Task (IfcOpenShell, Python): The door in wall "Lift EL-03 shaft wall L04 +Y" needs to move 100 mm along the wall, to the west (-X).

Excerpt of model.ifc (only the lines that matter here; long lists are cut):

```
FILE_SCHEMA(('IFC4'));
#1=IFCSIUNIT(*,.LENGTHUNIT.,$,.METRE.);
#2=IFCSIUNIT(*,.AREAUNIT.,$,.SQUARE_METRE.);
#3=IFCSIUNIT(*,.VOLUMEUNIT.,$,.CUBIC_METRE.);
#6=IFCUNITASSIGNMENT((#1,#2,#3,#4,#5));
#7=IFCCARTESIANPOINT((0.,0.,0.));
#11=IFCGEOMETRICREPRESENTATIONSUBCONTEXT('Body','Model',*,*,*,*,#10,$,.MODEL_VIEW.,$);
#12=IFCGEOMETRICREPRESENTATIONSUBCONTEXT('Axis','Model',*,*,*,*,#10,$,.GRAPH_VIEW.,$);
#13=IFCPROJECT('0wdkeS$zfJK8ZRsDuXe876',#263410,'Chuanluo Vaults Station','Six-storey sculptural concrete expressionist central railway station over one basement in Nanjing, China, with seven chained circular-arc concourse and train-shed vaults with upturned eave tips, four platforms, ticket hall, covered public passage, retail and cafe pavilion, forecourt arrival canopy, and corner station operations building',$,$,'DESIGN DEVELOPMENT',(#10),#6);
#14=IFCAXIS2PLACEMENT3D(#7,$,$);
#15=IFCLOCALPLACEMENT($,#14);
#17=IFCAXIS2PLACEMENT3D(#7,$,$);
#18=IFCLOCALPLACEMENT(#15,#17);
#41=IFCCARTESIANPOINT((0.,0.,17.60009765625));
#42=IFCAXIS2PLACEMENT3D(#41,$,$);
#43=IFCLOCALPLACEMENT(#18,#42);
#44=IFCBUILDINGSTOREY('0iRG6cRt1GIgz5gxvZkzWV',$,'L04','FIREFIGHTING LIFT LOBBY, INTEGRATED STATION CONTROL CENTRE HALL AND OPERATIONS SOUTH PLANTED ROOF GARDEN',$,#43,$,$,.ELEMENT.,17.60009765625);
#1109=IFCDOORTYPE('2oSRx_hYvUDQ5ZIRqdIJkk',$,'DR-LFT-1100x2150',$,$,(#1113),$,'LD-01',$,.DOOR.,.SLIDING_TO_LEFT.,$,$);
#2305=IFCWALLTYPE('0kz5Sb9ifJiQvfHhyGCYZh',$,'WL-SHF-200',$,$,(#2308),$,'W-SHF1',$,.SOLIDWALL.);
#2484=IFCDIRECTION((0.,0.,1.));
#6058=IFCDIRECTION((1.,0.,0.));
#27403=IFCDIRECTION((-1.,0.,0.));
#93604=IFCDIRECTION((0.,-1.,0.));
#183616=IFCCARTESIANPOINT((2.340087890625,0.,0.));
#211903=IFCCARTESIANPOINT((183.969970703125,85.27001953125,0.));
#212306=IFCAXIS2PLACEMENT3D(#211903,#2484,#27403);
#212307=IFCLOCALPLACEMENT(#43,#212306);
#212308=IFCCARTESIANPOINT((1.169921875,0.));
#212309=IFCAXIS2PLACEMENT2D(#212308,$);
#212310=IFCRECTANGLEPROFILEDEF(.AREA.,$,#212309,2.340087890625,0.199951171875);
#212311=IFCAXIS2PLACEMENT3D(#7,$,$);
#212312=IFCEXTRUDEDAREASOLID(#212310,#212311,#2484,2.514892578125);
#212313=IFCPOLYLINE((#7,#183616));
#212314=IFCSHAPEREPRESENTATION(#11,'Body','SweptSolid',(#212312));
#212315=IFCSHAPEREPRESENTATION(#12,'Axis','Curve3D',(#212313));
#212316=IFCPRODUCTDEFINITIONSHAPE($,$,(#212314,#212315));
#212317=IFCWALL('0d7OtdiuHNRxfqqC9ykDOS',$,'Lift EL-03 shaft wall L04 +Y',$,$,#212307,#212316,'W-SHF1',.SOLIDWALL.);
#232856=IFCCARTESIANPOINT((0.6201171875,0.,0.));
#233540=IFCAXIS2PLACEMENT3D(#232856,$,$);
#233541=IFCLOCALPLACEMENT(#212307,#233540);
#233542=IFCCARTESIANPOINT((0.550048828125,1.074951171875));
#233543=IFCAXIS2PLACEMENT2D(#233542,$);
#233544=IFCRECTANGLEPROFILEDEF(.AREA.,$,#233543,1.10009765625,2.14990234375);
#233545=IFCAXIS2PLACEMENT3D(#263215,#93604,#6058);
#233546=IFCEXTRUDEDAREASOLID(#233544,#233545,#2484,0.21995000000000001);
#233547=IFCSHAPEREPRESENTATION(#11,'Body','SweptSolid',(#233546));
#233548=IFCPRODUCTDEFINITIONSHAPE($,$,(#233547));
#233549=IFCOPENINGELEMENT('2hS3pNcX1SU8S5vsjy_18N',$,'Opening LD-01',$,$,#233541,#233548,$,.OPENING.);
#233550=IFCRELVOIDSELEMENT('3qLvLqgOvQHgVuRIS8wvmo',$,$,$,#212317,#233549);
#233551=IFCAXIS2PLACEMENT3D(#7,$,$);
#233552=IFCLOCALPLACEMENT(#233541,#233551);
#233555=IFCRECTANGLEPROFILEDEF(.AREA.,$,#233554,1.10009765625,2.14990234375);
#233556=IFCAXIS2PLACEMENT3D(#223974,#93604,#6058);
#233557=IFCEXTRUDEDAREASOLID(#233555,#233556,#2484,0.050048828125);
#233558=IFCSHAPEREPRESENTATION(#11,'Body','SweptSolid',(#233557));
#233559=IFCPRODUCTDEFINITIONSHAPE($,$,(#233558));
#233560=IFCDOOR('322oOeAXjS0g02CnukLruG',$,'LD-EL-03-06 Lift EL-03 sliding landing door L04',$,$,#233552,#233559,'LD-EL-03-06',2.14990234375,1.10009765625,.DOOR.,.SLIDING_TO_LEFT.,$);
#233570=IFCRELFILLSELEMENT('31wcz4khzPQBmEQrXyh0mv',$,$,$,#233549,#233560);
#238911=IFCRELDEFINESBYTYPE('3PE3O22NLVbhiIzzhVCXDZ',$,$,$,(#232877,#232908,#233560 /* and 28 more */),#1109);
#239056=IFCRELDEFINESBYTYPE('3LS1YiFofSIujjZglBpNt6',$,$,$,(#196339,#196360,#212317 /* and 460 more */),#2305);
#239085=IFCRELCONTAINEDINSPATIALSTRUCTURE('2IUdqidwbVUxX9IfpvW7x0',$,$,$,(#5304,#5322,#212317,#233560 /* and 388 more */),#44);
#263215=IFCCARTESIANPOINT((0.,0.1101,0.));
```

```python
import ifcopenshell
import ifcopenshell.api.geometry
import ifcopenshell.util.placement
import ifcopenshell.util.unit

model = ifcopenshell.open("model.ifc")
unit_scale = ifcopenshell.util.unit.calculate_unit_scale(model)

door = model.by_guid("322oOeAXjS0g02CnukLruG")
opening = door.FillsVoids[0].RelatingOpeningElement
wall = opening.VoidsElements[0].RelatingBuildingElement

wall_matrix = ifcopenshell.util.placement.get_local_placement(wall.ObjectPlacement)
shift = wall_matrix[:3, 0] * 0.1 / unit_scale
before = ifcopenshell.util.placement.get_local_placement(door.ObjectPlacement)[:3, 3].copy()

# The door is placed relative to its opening, so it follows when the opening moves.
matrix = ifcopenshell.util.placement.get_local_placement(opening.ObjectPlacement)
matrix[:3, 3] += shift
ifcopenshell.api.geometry.edit_object_placement(
    model, product=opening, matrix=matrix, is_si=False, should_transform_children=True
)

after = ifcopenshell.util.placement.get_local_placement(door.ObjectPlacement)[:3, 3]
print("door moved by", (after - before).round(3) + 0.0)

model.write("model_edited.ifc")
```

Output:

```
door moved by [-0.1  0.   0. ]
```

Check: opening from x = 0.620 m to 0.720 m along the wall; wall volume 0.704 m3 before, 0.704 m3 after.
